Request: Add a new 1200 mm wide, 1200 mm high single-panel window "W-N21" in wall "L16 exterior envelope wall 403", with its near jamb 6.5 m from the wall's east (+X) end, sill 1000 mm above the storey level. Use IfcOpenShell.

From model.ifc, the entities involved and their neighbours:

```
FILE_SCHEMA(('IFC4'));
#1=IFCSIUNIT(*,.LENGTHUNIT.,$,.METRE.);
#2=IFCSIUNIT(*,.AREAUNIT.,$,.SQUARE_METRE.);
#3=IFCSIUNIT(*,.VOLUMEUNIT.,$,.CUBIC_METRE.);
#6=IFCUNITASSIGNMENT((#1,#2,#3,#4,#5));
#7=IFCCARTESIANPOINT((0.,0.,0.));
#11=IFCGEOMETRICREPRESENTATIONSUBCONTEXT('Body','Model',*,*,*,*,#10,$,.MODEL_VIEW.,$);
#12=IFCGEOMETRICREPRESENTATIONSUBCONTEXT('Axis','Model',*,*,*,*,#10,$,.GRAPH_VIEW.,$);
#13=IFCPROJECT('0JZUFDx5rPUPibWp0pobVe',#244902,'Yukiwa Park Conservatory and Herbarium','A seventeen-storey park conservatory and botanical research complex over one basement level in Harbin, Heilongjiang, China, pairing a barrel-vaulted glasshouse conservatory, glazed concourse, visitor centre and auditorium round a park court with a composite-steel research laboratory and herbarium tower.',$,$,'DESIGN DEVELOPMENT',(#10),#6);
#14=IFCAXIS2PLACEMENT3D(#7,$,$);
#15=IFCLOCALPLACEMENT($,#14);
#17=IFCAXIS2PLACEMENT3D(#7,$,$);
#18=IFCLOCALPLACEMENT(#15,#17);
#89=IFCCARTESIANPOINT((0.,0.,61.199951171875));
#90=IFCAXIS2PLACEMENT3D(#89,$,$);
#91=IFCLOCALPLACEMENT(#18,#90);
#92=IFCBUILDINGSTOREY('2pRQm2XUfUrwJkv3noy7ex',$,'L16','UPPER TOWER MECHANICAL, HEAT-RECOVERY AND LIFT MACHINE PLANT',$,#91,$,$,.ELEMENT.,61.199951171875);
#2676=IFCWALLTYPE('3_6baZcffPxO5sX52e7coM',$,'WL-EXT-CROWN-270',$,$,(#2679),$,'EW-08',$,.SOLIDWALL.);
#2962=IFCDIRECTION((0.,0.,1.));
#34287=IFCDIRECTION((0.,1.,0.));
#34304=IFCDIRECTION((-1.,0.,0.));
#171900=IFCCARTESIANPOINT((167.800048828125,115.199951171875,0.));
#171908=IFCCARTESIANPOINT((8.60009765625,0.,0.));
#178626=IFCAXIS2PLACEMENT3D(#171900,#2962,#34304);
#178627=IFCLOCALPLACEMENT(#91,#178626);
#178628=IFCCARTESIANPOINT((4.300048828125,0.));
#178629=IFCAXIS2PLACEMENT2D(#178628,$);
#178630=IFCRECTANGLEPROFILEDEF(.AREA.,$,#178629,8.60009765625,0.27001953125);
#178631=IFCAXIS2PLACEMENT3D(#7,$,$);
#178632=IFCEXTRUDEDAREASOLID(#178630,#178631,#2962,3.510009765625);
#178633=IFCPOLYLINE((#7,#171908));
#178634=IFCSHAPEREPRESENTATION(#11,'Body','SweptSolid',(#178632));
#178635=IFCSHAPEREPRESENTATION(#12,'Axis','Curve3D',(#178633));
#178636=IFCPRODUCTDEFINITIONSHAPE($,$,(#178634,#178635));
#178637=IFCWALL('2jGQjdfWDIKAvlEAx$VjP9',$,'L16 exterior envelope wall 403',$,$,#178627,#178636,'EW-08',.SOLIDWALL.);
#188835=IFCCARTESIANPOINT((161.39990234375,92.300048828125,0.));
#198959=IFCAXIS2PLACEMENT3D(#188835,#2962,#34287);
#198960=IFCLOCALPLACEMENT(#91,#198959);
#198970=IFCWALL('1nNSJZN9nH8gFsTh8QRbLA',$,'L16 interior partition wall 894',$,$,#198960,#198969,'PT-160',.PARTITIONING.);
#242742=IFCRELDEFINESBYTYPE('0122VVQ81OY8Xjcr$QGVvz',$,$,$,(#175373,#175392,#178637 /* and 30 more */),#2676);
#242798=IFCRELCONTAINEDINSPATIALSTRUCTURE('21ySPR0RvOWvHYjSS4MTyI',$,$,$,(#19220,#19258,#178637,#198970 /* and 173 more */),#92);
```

```python
import numpy as np
import ifcopenshell
import ifcopenshell.api.feature
import ifcopenshell.api.geometry
import ifcopenshell.api.root
import ifcopenshell.api.spatial
import ifcopenshell.geom
import ifcopenshell.util.element
import ifcopenshell.util.placement
import ifcopenshell.util.representation
import ifcopenshell.util.shape
import ifcopenshell.util.unit

model = ifcopenshell.open("model.ifc")
unit_scale = ifcopenshell.util.unit.calculate_unit_scale(model)
settings = ifcopenshell.geom.settings()


def volume(element):
    """Net volume in cubic metres, openings subtracted."""
    shape = ifcopenshell.geom.create_shape(settings, element)
    return ifcopenshell.util.shape.get_volume(shape.geometry)


wall = model.by_guid("2jGQjdfWDIKAvlEAx$VjP9")
storey = ifcopenshell.util.element.get_container(wall, ifc_class="IfcBuildingStorey")
context = ifcopenshell.util.representation.get_context(model, "Model", "Body", "MODEL_VIEW")
before = volume(wall)

width, height, from_end, sill = 1.2, 1.2, 6.5, 1  # metres

# The wall runs along its own X axis, and the end named is its -X end.
wall_shape = ifcopenshell.geom.create_shape(settings, wall)
x, y, z = ifcopenshell.util.shape.get_vertices(wall_shape.geometry).T
start = x.min() + from_end
face, thickness = float(y.min()), float(y.max() - y.min())
wall_matrix = ifcopenshell.util.placement.get_local_placement(wall.ObjectPlacement)
level = ifcopenshell.util.placement.get_local_placement(storey.ObjectPlacement)[2, 3]


def in_wall(x, y):
    """Placement at x, y metres in the wall's axes, at sill height."""
    matrix = wall_matrix.copy()
    matrix[:, 3] = wall_matrix @ np.array([x / unit_scale, y / unit_scale, 0.0, 1.0])
    matrix[2, 3] = level + sill / unit_scale
    return matrix


# Opening: a box that overshoots both wall faces by 50 mm.
opening = ifcopenshell.api.root.create_entity(model, ifc_class="IfcOpeningElement", predefined_type="OPENING")
box = ifcopenshell.api.geometry.add_wall_representation(
    model, context=context, length=width, height=height, thickness=thickness + 0.1
)
ifcopenshell.api.geometry.assign_representation(model, product=opening, representation=box)
ifcopenshell.api.geometry.edit_object_placement(model, product=opening, matrix=in_wall(start, face - 0.05), is_si=False)
ifcopenshell.api.feature.add_feature(model, feature=opening, element=wall)

window = ifcopenshell.api.root.create_entity(model, ifc_class="IfcWindow", name="W-N21", predefined_type="WINDOW")
window.OverallWidth, window.OverallHeight = width / unit_scale, height / unit_scale
window.PartitioningType = "SINGLE_PANEL"
body = ifcopenshell.api.geometry.add_window_representation(
    model,
    context=context,
    overall_width=window.OverallWidth,
    overall_height=window.OverallHeight,
    partition_type="SINGLE_PANEL",
)
ifcopenshell.api.geometry.assign_representation(model, product=window, representation=body)
ifcopenshell.api.spatial.assign_container(model, products=[window], relating_structure=storey)
ifcopenshell.api.feature.add_filling(model, opening=opening, element=window)

# Centre the window in the wall's thickness.
ifcopenshell.api.geometry.edit_object_placement(model, product=window, matrix=in_wall(start, face), is_si=False)
window_shape = ifcopenshell.geom.create_shape(settings, window)
depth = ifcopenshell.util.shape.get_vertices(window_shape.geometry)[:, 1]
offset = face + thickness / 2 - (depth.min() + depth.max()) / 2
ifcopenshell.api.geometry.edit_object_placement(model, product=window, matrix=in_wall(start, offset), is_si=False)

after = volume(wall)

print(f"wall volume {before:.3f} -> {after:.3f} m3")

model.write("model_rev.ifc")
```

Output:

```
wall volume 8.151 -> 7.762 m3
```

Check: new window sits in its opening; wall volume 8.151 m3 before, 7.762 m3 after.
